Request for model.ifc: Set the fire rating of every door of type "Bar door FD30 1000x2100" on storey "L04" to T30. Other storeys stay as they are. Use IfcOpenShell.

First a look at what the model holds.

```python
import ifcopenshell
import ifcopenshell.util.element

model = ifcopenshell.open("model.ifc")
print(model.schema)
storey = next(s for s in model.by_type("IfcBuildingStorey") if s.Name == "L04")
doors = [e for e in ifcopenshell.util.element.get_decomposition(storey) if e.is_a("IfcDoor")]
seen = {}
for e in doors:
    element_type = ifcopenshell.util.element.get_type(e)
    key = (element_type.Name if element_type != e and element_type else None, ifcopenshell.util.element.get_pset(e, "Pset_DoorCommon", "FireRating"))
    seen[key] = seen.get(key, 0) + 1
for (name, value), count in sorted(seen.items(), key=str):
    print(count, "x", name, "|", value)
```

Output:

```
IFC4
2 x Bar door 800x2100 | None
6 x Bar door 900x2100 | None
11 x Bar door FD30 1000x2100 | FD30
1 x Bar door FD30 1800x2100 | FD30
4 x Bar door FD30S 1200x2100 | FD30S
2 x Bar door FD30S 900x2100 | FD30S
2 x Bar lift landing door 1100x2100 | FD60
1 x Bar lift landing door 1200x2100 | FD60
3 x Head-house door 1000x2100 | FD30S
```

```python
import ifcopenshell
import ifcopenshell.api.pset
import ifcopenshell.util.element

model = ifcopenshell.open("model.ifc")

storey = next(s for s in model.by_type("IfcBuildingStorey") if s.Name == "L04")
doors = [e for e in ifcopenshell.util.element.get_decomposition(storey) if e.is_a("IfcDoor")]

count = 0
for e in doors:
    element_type = ifcopenshell.util.element.get_type(e)
    if element_type in (None, e) or element_type.Name != "Bar door FD30 1000x2100":
        continue
    # add_pset returns the element's existing set when there is one.
    pset = ifcopenshell.api.pset.add_pset(model, product=e, name="Pset_DoorCommon")
    ifcopenshell.api.pset.edit_pset(model, pset=pset, properties={"FireRating": "T30"})
    count += 1

print(count, "doors updated")

model.write("model_v2.ifc")
```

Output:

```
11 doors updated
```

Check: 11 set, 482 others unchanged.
